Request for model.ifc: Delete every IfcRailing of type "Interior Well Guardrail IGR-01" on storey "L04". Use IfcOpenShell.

First a look at what the model holds.

```python
import ifcopenshell
import ifcopenshell.util.element

model = ifcopenshell.open("model.ifc")
print(model.schema)
storey = next(s for s in model.by_type("IfcBuildingStorey") if s.Name == "L04")
railings = [e for e in ifcopenshell.util.element.get_decomposition(storey) if e.is_a("IfcRailing")]
seen = {}
for e in railings:
    element_type = ifcopenshell.util.element.get_type(e)
    name = element_type.Name if element_type not in (None, e) else None
    seen[name] = seen.get(name, 0) + 1
for name, count in sorted(seen.items(), key=str):
    print(count, "x", name)
```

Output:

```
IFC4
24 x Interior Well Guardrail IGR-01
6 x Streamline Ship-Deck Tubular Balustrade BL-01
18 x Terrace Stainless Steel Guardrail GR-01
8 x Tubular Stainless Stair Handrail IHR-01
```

```python
import ifcopenshell
import ifcopenshell.api.root
import ifcopenshell.util.element

model = ifcopenshell.open("model.ifc")

storey = next(s for s in model.by_type("IfcBuildingStorey") if s.Name == "L04")
railings = [e for e in ifcopenshell.util.element.get_decomposition(storey) if e.is_a("IfcRailing")]
targets = [e for e in railings if (t := ifcopenshell.util.element.get_type(e)) not in (None, e) and t.Name == "Interior Well Guardrail IGR-01"]

for e in targets:
    ifcopenshell.api.root.remove_product(model, product=e)
print(len(targets), "removed")

model.write("model_v2.ifc")
```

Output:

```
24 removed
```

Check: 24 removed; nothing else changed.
